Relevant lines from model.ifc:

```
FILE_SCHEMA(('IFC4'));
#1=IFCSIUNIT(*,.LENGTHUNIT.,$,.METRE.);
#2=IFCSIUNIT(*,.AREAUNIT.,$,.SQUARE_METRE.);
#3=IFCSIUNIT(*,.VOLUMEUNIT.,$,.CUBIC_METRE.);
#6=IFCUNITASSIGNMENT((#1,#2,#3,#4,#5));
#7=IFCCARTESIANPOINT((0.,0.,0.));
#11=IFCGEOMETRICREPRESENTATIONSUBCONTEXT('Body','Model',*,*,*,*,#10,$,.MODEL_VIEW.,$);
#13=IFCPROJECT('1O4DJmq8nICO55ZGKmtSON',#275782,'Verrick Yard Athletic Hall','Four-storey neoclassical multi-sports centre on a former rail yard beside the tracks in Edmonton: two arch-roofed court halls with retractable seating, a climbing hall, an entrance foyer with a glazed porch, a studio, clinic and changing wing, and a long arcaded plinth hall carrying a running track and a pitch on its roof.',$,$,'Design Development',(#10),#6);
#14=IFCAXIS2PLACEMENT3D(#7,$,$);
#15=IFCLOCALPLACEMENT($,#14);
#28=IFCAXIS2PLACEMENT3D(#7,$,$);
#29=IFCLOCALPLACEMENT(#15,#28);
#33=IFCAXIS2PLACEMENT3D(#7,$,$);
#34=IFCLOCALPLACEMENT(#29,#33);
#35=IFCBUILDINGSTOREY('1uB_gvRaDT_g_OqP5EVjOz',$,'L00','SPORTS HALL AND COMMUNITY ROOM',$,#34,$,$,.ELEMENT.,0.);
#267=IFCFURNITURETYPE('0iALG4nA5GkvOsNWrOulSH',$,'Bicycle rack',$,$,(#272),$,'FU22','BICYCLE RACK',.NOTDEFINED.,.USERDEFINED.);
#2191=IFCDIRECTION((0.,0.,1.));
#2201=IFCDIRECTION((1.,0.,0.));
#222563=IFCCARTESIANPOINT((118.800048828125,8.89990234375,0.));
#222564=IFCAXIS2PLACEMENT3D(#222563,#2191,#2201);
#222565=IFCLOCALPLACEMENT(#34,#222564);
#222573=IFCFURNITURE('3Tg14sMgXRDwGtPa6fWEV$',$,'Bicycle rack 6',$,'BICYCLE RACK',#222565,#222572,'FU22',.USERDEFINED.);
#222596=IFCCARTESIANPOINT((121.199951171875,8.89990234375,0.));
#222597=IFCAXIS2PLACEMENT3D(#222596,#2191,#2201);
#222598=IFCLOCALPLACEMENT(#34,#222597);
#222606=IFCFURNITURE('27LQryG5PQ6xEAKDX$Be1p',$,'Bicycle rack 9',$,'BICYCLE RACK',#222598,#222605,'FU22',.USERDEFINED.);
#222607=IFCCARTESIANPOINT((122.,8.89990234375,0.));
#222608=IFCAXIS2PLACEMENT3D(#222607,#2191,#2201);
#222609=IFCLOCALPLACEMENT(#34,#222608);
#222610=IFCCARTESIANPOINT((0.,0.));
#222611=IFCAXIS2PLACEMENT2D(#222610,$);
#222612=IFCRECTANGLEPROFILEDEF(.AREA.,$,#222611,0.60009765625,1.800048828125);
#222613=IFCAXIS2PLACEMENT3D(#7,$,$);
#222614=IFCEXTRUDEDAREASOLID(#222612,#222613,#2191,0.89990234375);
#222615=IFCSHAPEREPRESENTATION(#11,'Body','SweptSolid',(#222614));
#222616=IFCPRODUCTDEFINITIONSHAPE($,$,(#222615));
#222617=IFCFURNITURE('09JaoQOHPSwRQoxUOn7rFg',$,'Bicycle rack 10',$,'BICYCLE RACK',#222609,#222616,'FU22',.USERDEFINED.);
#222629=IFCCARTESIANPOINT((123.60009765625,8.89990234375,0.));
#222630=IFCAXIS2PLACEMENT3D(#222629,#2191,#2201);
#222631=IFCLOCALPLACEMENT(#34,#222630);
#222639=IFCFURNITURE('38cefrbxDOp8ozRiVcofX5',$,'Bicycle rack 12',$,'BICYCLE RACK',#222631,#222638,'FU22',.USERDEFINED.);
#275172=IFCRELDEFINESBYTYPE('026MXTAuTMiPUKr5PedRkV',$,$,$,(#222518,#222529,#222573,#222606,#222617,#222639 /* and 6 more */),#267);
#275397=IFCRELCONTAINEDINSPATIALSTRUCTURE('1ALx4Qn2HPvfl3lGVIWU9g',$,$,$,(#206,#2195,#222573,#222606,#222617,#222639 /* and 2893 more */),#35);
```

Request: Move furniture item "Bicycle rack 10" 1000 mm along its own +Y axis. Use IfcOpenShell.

```python
import ifcopenshell
import ifcopenshell.api.geometry
import ifcopenshell.util.placement
import ifcopenshell.util.unit

model = ifcopenshell.open("model.ifc")
unit_scale = ifcopenshell.util.unit.calculate_unit_scale(model)

item = model.by_guid("09JaoQOHPSwRQoxUOn7rFg")
matrix = ifcopenshell.util.placement.get_local_placement(item.ObjectPlacement)
matrix[:3, 3] += matrix[:3, 1] * 1 / unit_scale
ifcopenshell.api.geometry.edit_object_placement(model, product=item, matrix=matrix, is_si=False)

print(ifcopenshell.util.placement.get_local_placement(item.ObjectPlacement).round(3) + 0.0)

model.write("model-out.ifc")
```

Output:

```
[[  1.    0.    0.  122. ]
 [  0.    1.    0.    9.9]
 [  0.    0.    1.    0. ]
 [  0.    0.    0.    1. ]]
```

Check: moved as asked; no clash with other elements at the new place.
